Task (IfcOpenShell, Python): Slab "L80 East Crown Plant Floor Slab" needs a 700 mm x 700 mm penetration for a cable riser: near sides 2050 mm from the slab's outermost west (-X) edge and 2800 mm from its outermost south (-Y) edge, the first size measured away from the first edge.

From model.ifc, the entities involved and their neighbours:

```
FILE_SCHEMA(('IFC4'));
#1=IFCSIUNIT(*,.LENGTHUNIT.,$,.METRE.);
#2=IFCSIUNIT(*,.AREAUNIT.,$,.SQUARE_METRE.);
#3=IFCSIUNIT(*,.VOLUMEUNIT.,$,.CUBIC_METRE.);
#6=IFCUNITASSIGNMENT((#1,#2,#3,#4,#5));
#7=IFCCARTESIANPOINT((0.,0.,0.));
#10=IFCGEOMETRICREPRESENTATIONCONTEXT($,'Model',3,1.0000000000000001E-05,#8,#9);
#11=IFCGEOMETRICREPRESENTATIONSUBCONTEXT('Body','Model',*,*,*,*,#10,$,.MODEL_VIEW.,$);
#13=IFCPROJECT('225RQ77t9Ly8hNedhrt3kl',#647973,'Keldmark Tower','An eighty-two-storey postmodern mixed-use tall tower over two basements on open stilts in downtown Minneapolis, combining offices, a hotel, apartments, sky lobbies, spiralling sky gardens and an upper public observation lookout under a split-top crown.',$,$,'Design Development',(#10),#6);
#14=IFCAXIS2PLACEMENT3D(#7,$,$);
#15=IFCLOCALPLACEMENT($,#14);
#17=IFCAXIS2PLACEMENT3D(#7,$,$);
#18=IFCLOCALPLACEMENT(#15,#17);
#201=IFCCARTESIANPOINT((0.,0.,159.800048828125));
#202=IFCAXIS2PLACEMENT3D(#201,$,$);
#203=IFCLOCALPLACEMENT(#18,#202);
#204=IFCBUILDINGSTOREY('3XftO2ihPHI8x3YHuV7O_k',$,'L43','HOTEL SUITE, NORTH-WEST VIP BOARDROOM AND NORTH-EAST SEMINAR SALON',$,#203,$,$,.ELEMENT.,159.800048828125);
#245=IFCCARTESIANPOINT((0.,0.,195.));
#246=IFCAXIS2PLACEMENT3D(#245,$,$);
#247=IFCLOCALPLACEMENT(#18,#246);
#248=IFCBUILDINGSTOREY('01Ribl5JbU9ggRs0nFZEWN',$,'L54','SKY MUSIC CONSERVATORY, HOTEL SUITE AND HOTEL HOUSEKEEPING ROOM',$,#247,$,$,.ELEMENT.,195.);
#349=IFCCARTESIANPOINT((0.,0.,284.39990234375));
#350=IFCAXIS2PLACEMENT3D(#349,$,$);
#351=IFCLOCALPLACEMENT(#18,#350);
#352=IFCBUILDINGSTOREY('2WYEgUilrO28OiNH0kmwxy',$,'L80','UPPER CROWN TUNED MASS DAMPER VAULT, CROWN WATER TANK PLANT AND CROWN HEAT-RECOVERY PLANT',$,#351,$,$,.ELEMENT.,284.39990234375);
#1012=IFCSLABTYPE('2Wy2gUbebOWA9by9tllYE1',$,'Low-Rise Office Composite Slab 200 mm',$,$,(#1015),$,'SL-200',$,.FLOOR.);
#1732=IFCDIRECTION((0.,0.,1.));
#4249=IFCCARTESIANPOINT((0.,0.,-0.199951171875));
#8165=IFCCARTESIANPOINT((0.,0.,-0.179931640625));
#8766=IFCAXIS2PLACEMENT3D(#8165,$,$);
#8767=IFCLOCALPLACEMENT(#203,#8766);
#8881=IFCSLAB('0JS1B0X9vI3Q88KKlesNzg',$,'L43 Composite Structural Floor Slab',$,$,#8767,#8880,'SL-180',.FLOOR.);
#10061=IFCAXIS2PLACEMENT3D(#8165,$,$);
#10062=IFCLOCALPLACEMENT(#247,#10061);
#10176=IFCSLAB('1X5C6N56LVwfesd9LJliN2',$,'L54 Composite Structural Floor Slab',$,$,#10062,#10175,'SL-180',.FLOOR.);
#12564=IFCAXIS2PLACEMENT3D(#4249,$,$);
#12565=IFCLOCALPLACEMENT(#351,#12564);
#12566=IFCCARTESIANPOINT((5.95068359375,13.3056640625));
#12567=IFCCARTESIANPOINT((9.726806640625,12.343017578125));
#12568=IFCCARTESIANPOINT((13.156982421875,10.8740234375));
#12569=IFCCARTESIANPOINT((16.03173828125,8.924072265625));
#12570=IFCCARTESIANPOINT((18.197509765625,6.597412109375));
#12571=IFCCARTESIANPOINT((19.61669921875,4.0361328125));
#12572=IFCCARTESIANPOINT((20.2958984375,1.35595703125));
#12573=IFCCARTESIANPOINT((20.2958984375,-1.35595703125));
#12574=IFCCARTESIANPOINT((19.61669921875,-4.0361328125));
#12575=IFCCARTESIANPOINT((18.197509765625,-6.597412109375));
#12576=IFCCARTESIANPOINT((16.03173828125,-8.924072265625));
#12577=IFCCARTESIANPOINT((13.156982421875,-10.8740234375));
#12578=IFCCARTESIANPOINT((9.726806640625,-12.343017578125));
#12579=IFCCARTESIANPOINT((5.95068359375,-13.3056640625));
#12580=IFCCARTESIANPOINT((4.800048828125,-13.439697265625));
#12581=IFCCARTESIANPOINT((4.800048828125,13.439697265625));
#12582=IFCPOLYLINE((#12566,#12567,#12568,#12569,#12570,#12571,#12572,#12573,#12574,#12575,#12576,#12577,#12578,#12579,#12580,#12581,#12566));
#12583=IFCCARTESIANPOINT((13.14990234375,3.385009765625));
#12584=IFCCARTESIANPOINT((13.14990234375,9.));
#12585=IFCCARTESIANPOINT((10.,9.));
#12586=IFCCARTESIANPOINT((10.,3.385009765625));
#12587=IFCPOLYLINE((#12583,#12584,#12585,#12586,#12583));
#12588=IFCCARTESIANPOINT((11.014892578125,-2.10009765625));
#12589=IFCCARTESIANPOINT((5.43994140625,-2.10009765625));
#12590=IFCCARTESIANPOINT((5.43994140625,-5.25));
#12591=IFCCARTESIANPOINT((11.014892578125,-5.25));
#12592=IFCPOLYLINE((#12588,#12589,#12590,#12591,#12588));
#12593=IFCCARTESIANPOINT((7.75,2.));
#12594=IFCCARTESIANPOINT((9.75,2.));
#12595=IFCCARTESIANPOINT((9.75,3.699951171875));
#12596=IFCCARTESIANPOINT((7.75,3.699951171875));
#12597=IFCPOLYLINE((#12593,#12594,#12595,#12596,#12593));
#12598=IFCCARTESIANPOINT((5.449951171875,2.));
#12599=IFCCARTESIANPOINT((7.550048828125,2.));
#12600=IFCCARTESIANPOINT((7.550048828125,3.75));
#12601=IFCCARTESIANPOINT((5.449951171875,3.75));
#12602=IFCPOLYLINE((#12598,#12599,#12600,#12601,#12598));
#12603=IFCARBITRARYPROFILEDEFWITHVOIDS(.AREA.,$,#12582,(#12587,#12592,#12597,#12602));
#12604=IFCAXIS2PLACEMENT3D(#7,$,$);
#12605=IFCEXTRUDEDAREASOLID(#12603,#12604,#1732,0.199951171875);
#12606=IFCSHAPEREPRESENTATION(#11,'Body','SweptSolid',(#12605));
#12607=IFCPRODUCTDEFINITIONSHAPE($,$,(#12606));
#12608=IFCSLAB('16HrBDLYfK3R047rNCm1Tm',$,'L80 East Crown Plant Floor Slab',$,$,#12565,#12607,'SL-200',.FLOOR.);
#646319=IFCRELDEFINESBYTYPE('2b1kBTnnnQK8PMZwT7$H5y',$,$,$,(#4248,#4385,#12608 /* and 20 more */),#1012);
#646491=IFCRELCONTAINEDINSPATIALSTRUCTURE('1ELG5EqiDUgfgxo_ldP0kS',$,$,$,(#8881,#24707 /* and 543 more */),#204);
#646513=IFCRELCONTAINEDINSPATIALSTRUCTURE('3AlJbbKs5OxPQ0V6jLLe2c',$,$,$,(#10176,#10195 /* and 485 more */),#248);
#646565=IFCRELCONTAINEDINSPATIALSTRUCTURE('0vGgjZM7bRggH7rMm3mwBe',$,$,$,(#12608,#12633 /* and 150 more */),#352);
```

```python
import numpy as np
import ifcopenshell
import ifcopenshell.api.feature
import ifcopenshell.api.geometry
import ifcopenshell.api.root
import ifcopenshell.geom
import ifcopenshell.util.placement
import ifcopenshell.util.representation
import ifcopenshell.util.shape
import ifcopenshell.util.unit

model = ifcopenshell.open("model.ifc")
unit_scale = ifcopenshell.util.unit.calculate_unit_scale(model)
settings = ifcopenshell.geom.settings()


def volume(element):
    """Net volume in cubic metres, openings subtracted."""
    shape = ifcopenshell.geom.create_shape(settings, element)
    return ifcopenshell.util.shape.get_volume(shape.geometry)


slab = model.by_id(12608)
before = volume(slab)

# Extent in the slab's own axes, in metres. The edges named are its -X and -Y sides.
slab_shape = ifcopenshell.geom.create_shape(settings, slab)
vertices = ifcopenshell.util.shape.get_vertices(slab_shape.geometry)
x_min, y_min, bottom = vertices.min(axis=0)
top = vertices[:, 2].max()

opening = ifcopenshell.api.root.create_entity(model, ifc_class="IfcOpeningElement", name="Cable riser opening", predefined_type="OPENING")
context = ifcopenshell.util.representation.get_context(model, "Model", "Body", "MODEL_VIEW")
width, depth = 0.7, 0.7
outline = [(0.0, 0.0), (width, 0.0), (width, depth), (0.0, depth), (0.0, 0.0)]
# Overshoot both faces by 50 mm so the cut is clean.
shape = ifcopenshell.api.geometry.add_slab_representation(
    model, context=context, depth=top - bottom + 0.1, polyline=outline
)
ifcopenshell.api.geometry.assign_representation(model, product=opening, representation=shape)

matrix = ifcopenshell.util.placement.get_local_placement(slab.ObjectPlacement)
matrix[:, 3] = matrix @ np.append(np.array([x_min + 2.05, y_min + 2.8, bottom - 0.05]) / unit_scale, 1.0)
ifcopenshell.api.geometry.edit_object_placement(model, product=opening, matrix=matrix, is_si=False)
ifcopenshell.api.feature.add_feature(model, feature=opening, element=slab)

after = volume(slab)

print(f"slab volume {before:.3f} -> {after:.3f} m3")

model.write("model_v2.ifc")
```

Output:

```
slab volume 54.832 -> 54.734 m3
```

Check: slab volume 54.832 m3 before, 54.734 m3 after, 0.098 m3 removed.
